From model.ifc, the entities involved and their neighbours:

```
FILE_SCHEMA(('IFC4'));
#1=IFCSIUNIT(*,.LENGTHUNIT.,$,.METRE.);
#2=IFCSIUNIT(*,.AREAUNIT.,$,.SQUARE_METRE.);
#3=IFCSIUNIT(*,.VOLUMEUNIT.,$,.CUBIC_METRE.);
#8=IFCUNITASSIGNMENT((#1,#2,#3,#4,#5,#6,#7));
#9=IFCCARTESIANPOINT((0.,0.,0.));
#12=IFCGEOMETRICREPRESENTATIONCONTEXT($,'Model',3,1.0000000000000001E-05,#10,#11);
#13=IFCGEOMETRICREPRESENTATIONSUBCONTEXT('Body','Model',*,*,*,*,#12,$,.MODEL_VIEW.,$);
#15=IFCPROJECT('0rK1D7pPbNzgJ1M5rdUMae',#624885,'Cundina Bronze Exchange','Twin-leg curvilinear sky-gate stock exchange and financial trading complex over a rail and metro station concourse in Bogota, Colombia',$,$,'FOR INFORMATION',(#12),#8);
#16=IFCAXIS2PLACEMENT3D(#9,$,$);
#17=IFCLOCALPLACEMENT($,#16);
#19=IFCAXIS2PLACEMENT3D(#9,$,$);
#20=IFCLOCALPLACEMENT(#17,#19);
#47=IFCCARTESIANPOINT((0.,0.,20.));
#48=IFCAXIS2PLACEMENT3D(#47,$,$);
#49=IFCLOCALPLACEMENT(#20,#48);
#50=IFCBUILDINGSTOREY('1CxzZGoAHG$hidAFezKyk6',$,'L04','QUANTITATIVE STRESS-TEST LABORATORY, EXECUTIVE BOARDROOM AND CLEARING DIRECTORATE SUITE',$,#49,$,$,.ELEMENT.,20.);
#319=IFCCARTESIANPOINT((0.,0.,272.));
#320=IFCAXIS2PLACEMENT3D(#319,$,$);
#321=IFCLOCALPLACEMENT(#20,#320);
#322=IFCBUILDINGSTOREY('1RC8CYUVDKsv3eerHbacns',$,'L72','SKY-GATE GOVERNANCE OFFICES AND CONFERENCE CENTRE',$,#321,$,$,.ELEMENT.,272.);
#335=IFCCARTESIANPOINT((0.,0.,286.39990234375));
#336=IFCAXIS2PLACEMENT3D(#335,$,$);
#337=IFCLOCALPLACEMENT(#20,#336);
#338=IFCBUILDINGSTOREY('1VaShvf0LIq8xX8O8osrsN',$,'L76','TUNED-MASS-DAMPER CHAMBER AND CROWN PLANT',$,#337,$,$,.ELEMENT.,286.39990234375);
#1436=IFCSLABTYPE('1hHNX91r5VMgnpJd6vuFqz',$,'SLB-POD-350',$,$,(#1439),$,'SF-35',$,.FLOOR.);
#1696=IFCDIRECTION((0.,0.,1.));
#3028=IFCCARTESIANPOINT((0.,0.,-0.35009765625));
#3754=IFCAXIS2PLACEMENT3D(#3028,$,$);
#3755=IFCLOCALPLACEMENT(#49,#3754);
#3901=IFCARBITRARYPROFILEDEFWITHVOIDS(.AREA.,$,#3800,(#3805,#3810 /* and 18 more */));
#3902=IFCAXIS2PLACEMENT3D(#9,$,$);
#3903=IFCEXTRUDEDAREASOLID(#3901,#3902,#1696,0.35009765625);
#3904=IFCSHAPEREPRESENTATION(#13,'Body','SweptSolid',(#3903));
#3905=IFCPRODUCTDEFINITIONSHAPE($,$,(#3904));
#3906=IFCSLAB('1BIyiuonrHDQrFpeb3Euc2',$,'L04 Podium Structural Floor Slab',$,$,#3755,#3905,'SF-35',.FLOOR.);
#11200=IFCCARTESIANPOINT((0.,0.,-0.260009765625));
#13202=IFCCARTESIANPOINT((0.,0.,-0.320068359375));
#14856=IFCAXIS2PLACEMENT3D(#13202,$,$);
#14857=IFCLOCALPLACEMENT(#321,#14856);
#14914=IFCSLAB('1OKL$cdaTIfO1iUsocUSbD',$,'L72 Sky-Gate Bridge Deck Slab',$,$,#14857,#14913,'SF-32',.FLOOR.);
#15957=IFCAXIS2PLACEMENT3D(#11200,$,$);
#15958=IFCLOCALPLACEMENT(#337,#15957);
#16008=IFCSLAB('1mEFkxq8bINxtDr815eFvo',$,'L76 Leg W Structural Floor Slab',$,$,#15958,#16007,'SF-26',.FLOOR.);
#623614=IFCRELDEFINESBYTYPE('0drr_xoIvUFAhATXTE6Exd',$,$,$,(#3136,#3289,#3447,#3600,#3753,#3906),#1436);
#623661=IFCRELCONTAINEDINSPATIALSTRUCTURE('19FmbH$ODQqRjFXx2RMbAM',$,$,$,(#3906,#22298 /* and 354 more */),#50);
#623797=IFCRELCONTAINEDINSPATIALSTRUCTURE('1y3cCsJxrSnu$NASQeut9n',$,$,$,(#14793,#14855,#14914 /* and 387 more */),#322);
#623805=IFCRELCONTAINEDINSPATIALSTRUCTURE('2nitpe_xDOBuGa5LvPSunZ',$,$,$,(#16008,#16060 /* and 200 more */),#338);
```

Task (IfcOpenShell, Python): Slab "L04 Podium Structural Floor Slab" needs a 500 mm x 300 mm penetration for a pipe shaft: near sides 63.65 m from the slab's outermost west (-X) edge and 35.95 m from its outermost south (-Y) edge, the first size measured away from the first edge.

```python
import numpy as np
import ifcopenshell
import ifcopenshell.api.feature
import ifcopenshell.api.geometry
import ifcopenshell.api.root
import ifcopenshell.geom
import ifcopenshell.util.placement
import ifcopenshell.util.representation
import ifcopenshell.util.shape
import ifcopenshell.util.unit

model = ifcopenshell.open("model.ifc")
unit_scale = ifcopenshell.util.unit.calculate_unit_scale(model)
settings = ifcopenshell.geom.settings()


def volume(element):
    """Net volume in cubic metres, openings subtracted."""
    shape = ifcopenshell.geom.create_shape(settings, element)
    return ifcopenshell.util.shape.get_volume(shape.geometry)


slab = model.by_guid("1BIyiuonrHDQrFpeb3Euc2")
before = volume(slab)

# Extent in the slab's own axes, in metres. The edges named are its -X and -Y sides.
slab_shape = ifcopenshell.geom.create_shape(settings, slab)
vertices = ifcopenshell.util.shape.get_vertices(slab_shape.geometry)
x_min, y_min, bottom = vertices.min(axis=0)
top = vertices[:, 2].max()

opening = ifcopenshell.api.root.create_entity(model, ifc_class="IfcOpeningElement", name="Pipe shaft opening", predefined_type="OPENING")
context = ifcopenshell.util.representation.get_context(model, "Model", "Body", "MODEL_VIEW")
width, depth = 0.5, 0.3
outline = [(0.0, 0.0), (width, 0.0), (width, depth), (0.0, depth), (0.0, 0.0)]
# Overshoot both faces by 50 mm so the cut is clean.
shape = ifcopenshell.api.geometry.add_slab_representation(
    model, context=context, depth=top - bottom + 0.1, polyline=outline
)
ifcopenshell.api.geometry.assign_representation(model, product=opening, representation=shape)

matrix = ifcopenshell.util.placement.get_local_placement(slab.ObjectPlacement)
matrix[:, 3] = matrix @ np.append(np.array([x_min + 63.65, y_min + 35.95, bottom - 0.05]) / unit_scale, 1.0)
ifcopenshell.api.geometry.edit_object_placement(model, product=opening, matrix=matrix, is_si=False)
ifcopenshell.api.feature.add_feature(model, feature=opening, element=slab)

after = volume(slab)

print(f"slab volume {before:.3f} -> {after:.3f} m3")

model.write("model_rev.ifc")
```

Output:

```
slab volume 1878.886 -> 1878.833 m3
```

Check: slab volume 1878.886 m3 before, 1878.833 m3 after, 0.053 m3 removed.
